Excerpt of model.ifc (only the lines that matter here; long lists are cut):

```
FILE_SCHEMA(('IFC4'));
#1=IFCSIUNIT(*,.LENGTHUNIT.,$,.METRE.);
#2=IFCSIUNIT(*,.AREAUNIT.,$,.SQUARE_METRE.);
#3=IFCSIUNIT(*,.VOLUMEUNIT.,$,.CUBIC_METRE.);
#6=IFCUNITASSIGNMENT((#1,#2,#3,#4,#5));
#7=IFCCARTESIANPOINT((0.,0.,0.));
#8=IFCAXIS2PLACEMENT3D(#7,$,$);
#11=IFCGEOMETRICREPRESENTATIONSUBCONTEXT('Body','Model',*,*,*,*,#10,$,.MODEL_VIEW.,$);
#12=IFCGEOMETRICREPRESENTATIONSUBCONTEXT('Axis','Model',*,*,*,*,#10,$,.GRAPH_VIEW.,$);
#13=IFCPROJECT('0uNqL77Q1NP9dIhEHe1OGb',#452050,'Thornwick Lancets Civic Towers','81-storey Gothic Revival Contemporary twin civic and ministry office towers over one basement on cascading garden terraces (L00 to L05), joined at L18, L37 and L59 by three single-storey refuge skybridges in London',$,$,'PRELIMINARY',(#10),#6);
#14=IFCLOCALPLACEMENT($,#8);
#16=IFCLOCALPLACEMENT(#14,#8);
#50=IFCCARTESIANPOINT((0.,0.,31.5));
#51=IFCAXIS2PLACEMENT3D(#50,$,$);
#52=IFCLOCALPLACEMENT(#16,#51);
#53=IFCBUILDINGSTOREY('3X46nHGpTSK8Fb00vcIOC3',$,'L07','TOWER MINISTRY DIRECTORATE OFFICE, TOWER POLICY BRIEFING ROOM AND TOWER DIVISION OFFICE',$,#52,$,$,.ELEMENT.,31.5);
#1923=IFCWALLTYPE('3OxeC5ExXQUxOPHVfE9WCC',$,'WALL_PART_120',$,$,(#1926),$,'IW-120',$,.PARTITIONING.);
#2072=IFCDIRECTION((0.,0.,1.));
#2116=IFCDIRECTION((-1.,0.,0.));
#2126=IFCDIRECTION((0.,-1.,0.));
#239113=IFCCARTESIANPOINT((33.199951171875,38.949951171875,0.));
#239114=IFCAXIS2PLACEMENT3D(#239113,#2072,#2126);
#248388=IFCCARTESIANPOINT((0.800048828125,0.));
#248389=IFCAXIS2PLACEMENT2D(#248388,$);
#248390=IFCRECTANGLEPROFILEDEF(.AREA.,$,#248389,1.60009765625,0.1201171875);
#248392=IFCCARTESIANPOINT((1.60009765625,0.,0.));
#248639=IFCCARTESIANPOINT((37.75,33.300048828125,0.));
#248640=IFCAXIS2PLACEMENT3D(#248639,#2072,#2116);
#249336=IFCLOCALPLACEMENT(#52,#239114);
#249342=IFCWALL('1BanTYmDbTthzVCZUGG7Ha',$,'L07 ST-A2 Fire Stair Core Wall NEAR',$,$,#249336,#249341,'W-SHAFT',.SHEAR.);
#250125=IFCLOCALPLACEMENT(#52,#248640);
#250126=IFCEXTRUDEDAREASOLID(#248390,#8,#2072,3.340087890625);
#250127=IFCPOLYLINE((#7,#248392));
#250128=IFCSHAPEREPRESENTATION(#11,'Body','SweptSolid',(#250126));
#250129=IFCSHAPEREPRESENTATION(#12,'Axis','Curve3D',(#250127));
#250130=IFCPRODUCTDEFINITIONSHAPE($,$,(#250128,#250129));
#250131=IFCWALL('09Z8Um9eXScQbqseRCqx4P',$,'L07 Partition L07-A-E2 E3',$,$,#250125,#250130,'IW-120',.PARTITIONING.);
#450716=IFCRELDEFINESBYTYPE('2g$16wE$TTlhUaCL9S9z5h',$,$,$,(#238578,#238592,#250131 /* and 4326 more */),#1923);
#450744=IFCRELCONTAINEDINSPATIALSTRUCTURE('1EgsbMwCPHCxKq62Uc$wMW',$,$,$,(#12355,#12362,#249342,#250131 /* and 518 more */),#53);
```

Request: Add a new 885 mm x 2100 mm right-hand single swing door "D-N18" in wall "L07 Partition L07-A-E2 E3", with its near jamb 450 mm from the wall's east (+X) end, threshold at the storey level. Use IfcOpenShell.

```python
import numpy as np
import ifcopenshell
import ifcopenshell.api.feature
import ifcopenshell.api.geometry
import ifcopenshell.api.root
import ifcopenshell.api.spatial
import ifcopenshell.geom
import ifcopenshell.util.element
import ifcopenshell.util.placement
import ifcopenshell.util.representation
import ifcopenshell.util.shape
import ifcopenshell.util.unit

model = ifcopenshell.open("model.ifc")
unit_scale = ifcopenshell.util.unit.calculate_unit_scale(model)
settings = ifcopenshell.geom.settings()


def volume(element):
    """Net volume in cubic metres, openings subtracted."""
    shape = ifcopenshell.geom.create_shape(settings, element)
    return ifcopenshell.util.shape.get_volume(shape.geometry)


wall = model.by_guid("09Z8Um9eXScQbqseRCqx4P")
storey = ifcopenshell.util.element.get_container(wall, ifc_class="IfcBuildingStorey")
context = ifcopenshell.util.representation.get_context(model, "Model", "Body", "MODEL_VIEW")
before = volume(wall)

width, height, from_end, sill = 0.885, 2.1, 0.45, 0.0  # metres

# The wall runs along its own X axis, and the end named is its -X end.
wall_shape = ifcopenshell.geom.create_shape(settings, wall)
x, y, z = ifcopenshell.util.shape.get_vertices(wall_shape.geometry).T
start = x.min() + from_end
face, thickness = float(y.min()), float(y.max() - y.min())
wall_matrix = ifcopenshell.util.placement.get_local_placement(wall.ObjectPlacement)
level = ifcopenshell.util.placement.get_local_placement(storey.ObjectPlacement)[2, 3]


def in_wall(x, y):
    """Placement at x, y metres in the wall's axes, at sill height."""
    matrix = wall_matrix.copy()
    matrix[:, 3] = wall_matrix @ np.array([x / unit_scale, y / unit_scale, 0.0, 1.0])
    matrix[2, 3] = level + sill / unit_scale
    return matrix


# Opening: a box that overshoots both wall faces by 50 mm.
opening = ifcopenshell.api.root.create_entity(model, ifc_class="IfcOpeningElement", predefined_type="OPENING")
box = ifcopenshell.api.geometry.add_wall_representation(
    model, context=context, length=width, height=height, thickness=thickness + 0.1
)
ifcopenshell.api.geometry.assign_representation(model, product=opening, representation=box)
ifcopenshell.api.geometry.edit_object_placement(model, product=opening, matrix=in_wall(start, face - 0.05), is_si=False)
ifcopenshell.api.feature.add_feature(model, feature=opening, element=wall)

door = ifcopenshell.api.root.create_entity(model, ifc_class="IfcDoor", name="D-N18", predefined_type="DOOR")
door.OverallWidth, door.OverallHeight = width / unit_scale, height / unit_scale
door.OperationType = "SINGLE_SWING_RIGHT"
body = ifcopenshell.api.geometry.add_door_representation(
    model,
    context=context,
    overall_width=door.OverallWidth,
    overall_height=door.OverallHeight,
    operation_type="SINGLE_SWING_RIGHT",
    lining_properties={"LiningDepth": thickness / unit_scale, "ThresholdDepth": thickness / unit_scale},
)
ifcopenshell.api.geometry.assign_representation(model, product=door, representation=body)
ifcopenshell.api.spatial.assign_container(model, products=[door], relating_structure=storey)
ifcopenshell.api.feature.add_filling(model, opening=opening, element=door)

# The lining spans the wall, so the door starts at the wall face.
ifcopenshell.api.geometry.edit_object_placement(model, product=door, matrix=in_wall(start, face), is_si=False)

after = volume(wall)

print(f"wall volume {before:.3f} -> {after:.3f} m3")

model.write("model_updated.ifc")
```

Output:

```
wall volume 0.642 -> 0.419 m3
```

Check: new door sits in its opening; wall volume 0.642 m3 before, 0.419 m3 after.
